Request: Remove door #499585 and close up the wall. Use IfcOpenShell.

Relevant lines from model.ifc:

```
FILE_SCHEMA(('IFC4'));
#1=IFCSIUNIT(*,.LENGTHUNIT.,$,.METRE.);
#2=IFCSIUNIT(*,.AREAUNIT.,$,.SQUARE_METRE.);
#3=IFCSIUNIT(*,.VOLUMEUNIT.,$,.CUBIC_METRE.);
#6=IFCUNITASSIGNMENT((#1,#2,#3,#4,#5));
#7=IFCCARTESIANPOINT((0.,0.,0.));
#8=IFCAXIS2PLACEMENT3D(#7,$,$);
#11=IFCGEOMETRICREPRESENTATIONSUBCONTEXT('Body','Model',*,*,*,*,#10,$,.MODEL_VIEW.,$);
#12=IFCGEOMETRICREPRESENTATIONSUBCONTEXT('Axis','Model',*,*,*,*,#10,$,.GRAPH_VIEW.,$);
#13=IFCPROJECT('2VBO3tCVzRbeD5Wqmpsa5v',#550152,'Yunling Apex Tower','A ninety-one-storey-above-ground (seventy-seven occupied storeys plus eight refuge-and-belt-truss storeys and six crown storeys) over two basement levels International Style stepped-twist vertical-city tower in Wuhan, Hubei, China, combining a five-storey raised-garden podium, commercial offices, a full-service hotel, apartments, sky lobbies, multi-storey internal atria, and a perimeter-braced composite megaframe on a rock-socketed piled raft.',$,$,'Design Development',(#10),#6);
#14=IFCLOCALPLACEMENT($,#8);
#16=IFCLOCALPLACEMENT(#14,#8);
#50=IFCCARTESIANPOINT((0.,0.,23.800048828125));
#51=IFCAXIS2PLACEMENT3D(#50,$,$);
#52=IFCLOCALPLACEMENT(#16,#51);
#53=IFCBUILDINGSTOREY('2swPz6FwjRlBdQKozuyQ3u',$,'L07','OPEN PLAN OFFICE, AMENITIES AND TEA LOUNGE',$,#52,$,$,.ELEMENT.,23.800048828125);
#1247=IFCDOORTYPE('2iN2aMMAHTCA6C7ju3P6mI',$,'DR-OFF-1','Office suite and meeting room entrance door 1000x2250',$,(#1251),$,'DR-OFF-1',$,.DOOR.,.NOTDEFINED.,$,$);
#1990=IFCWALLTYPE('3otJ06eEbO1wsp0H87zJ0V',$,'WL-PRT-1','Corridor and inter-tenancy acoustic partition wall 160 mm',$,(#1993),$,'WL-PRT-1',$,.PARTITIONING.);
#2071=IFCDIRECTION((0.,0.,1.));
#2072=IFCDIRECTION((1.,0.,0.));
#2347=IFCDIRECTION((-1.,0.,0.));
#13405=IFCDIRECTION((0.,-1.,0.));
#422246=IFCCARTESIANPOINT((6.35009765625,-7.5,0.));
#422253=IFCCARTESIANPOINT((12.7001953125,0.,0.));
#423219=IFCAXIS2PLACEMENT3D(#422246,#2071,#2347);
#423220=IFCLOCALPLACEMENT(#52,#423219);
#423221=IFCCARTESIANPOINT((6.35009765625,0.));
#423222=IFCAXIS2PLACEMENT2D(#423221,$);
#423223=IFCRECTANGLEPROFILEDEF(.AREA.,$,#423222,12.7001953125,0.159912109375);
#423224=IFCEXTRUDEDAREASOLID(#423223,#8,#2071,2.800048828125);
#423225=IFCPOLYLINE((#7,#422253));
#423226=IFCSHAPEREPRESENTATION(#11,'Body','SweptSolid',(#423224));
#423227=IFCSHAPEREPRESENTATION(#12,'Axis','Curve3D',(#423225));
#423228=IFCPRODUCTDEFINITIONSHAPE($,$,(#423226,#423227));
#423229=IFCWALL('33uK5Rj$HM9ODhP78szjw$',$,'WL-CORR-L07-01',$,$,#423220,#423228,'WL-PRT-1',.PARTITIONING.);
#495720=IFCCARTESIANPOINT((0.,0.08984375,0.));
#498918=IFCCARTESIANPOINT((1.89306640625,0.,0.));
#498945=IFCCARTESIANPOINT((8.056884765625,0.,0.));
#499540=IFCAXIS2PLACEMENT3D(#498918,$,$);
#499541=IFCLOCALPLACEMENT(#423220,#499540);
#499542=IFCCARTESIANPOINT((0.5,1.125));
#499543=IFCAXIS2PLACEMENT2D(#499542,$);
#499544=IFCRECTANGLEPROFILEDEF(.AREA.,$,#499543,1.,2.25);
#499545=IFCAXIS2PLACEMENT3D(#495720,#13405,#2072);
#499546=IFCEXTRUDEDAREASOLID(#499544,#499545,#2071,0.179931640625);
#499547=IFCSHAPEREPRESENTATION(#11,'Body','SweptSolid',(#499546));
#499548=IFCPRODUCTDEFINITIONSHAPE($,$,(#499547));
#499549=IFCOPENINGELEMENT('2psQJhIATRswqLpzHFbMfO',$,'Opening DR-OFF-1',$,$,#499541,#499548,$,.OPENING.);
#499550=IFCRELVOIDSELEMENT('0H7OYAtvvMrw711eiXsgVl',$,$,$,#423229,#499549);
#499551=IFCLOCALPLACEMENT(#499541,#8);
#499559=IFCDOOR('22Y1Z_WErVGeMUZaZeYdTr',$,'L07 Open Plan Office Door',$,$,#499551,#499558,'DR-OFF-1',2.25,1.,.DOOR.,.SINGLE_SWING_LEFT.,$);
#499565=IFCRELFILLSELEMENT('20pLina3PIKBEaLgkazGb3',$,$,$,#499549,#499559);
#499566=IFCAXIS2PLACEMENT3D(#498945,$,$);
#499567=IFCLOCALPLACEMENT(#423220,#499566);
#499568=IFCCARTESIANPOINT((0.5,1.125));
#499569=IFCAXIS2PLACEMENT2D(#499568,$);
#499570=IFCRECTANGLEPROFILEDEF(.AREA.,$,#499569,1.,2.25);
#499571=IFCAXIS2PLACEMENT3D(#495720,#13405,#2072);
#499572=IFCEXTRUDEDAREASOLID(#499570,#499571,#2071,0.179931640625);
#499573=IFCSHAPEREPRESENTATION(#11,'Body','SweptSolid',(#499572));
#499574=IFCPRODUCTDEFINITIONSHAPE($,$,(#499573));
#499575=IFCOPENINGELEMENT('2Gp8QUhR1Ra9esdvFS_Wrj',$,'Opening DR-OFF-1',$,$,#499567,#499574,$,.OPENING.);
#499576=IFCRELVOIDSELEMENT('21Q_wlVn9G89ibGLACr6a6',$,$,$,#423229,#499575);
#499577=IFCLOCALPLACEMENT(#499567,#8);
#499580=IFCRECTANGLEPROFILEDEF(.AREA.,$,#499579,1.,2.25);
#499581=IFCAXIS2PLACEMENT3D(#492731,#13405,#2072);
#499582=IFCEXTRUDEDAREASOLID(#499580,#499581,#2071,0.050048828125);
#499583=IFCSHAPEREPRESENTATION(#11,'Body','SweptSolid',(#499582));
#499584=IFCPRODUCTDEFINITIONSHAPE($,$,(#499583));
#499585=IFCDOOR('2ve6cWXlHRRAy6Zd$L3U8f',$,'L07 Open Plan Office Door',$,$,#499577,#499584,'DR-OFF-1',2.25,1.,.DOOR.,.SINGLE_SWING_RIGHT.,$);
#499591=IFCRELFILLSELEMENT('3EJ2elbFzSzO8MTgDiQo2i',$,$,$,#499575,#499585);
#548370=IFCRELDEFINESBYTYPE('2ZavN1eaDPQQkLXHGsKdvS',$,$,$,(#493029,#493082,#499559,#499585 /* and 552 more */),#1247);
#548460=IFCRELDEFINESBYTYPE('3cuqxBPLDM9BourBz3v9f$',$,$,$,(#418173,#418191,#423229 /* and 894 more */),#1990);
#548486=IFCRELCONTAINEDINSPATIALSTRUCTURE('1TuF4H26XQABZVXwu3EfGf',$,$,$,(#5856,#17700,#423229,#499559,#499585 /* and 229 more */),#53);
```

```python
import ifcopenshell
import ifcopenshell.api.feature
import ifcopenshell.api.root
import ifcopenshell.geom
import ifcopenshell.util.shape

model = ifcopenshell.open("model.ifc")
settings = ifcopenshell.geom.settings()


def volume(element):
    """Net volume in cubic metres, openings subtracted."""
    shape = ifcopenshell.geom.create_shape(settings, element)
    return ifcopenshell.util.shape.get_volume(shape.geometry)


door = model.by_guid("2ve6cWXlHRRAy6Zd$L3U8f")
opening = door.FillsVoids[0].RelatingOpeningElement
wall = opening.VoidsElements[0].RelatingBuildingElement
before = volume(wall)

ifcopenshell.api.root.remove_product(model, product=door)
ifcopenshell.api.feature.remove_feature(model, feature=opening)

after = volume(wall)

print(f"wall volume {before:.3f} -> {after:.3f} m3")

model.write("model_v2.ifc")
```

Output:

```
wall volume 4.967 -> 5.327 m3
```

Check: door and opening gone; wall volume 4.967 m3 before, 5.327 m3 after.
